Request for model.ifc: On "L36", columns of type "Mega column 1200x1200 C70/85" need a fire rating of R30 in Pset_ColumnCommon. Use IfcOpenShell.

First a look at what the model holds.

```python
import ifcopenshell
import ifcopenshell.util.element

model = ifcopenshell.open("model.ifc")
print(model.schema)
storey = next(s for s in model.by_type("IfcBuildingStorey") if s.Name == "L36")
columns = [e for e in ifcopenshell.util.element.get_decomposition(storey) if e.is_a("IfcColumn")]
seen = {}
for e in columns:
    element_type = ifcopenshell.util.element.get_type(e)
    key = (element_type.Name if element_type != e and element_type else None, ifcopenshell.util.element.get_pset(e, "Pset_ColumnCommon", "FireRating"))
    seen[key] = seen.get(key, 0) + 1
for (name, value), count in sorted(seen.items(), key=str):
    print(count, "x", name, "|", value)
```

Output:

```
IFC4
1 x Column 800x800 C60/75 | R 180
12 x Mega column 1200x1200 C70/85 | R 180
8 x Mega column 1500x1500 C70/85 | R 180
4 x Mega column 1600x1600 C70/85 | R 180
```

```python
import ifcopenshell
import ifcopenshell.api.pset
import ifcopenshell.util.element

model = ifcopenshell.open("model.ifc")

storey = next(s for s in model.by_type("IfcBuildingStorey") if s.Name == "L36")
columns = [e for e in ifcopenshell.util.element.get_decomposition(storey) if e.is_a("IfcColumn")]

count = 0
for e in columns:
    element_type = ifcopenshell.util.element.get_type(e)
    if element_type in (None, e) or element_type.Name != "Mega column 1200x1200 C70/85":
        continue
    found = ifcopenshell.util.element.get_pset(e, "Pset_ColumnCommon", should_inherit=False)
    if found:
        pset = model.by_id(found["id"])
        if len(ifcopenshell.util.element.get_elements_by_pset(pset)) > 1:
            pset = ifcopenshell.api.pset.unshare_pset(model, products=[e], pset=pset)[0]
    else:
        pset = ifcopenshell.api.pset.add_pset(model, product=e, name="Pset_ColumnCommon")
    ifcopenshell.api.pset.edit_pset(model, pset=pset, properties={"FireRating": "R30"})
    count += 1

print(count, "columns updated")

model.write("model_rev.ifc")
```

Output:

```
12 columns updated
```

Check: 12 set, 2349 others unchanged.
